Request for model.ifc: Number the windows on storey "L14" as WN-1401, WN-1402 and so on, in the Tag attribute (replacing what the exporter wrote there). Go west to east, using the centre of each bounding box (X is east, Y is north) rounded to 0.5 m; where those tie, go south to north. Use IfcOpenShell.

First a look at what the model holds.

```python
import ifcopenshell
import ifcopenshell.util.element
import ifcopenshell.util.placement

model = ifcopenshell.open("model.ifc")
print(model.schema)
storey = next(s for s in model.by_type("IfcBuildingStorey") if s.Name == "L14")
windows = [e for e in ifcopenshell.util.element.get_decomposition(storey) if e.is_a("IfcWindow")]
for e in sorted(windows, key=lambda e: e.id()):
    origin = ifcopenshell.util.placement.get_local_placement(e.ObjectPlacement)[:3, 3]
    print(e.id(), e.Tag, e.Name, origin.round(2) + 0.0, sep=" | ")
```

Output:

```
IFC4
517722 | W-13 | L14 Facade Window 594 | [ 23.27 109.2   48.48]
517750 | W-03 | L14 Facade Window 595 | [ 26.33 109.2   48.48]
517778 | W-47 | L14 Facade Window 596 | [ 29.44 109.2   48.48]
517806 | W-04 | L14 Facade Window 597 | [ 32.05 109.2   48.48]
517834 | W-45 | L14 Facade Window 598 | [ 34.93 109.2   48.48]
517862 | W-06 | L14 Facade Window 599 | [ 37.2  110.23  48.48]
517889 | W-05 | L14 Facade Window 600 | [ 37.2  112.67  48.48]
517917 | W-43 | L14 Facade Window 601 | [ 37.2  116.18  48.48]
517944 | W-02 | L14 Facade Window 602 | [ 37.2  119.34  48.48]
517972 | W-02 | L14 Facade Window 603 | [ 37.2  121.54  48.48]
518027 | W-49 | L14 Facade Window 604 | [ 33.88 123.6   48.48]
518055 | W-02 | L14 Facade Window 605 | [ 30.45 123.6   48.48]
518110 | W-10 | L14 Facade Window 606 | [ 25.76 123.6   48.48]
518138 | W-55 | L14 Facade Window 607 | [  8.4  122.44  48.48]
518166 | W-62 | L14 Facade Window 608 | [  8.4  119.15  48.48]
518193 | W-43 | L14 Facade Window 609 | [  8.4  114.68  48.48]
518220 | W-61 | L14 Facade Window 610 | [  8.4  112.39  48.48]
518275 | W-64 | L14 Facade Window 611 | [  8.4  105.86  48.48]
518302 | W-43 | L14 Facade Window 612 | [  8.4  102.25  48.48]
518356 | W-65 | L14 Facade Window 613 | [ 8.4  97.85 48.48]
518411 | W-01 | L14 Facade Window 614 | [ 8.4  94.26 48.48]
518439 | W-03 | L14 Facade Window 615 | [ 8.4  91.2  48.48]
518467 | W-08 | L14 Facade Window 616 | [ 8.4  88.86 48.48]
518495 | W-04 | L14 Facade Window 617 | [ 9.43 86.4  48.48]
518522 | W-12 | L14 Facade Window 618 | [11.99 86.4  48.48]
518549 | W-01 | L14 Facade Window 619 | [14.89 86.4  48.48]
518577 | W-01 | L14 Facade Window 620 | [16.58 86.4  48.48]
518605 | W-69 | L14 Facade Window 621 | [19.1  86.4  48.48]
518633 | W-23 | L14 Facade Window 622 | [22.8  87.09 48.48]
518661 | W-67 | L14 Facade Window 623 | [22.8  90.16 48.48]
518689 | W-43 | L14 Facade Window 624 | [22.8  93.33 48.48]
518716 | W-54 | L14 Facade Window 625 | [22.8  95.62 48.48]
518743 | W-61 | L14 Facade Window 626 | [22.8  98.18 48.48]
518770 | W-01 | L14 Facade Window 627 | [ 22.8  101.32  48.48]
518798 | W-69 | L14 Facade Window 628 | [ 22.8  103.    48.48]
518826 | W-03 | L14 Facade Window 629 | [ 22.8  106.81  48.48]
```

```python
import ifcopenshell
import ifcopenshell.geom
import ifcopenshell.util.element
import ifcopenshell.util.shape

model = ifcopenshell.open("model.ifc")
settings = ifcopenshell.geom.settings()
settings.set("use-world-coords", True)


def centre(element):
    shape = ifcopenshell.geom.create_shape(settings, element)
    return ifcopenshell.util.shape.get_bbox_centroid(shape.geometry)


storey = next(s for s in model.by_type("IfcBuildingStorey") if s.Name == "L14")
windows = [e for e in ifcopenshell.util.element.get_decomposition(storey) if e.is_a("IfcWindow")]

# Insertion points can sit at a corner or the storey origin, so sort by the geometry (in metres).
centres = {e: centre(e) for e in windows}
windows.sort(key=lambda e: (round(centres[e][0] / 0.5), centres[e][1]))

for i, e in enumerate(windows, start=1):
    number = f"WN-14{i:02d}"
    e.Tag = number
    print(e.id(), number)

model.write("model_edited.ifc")
```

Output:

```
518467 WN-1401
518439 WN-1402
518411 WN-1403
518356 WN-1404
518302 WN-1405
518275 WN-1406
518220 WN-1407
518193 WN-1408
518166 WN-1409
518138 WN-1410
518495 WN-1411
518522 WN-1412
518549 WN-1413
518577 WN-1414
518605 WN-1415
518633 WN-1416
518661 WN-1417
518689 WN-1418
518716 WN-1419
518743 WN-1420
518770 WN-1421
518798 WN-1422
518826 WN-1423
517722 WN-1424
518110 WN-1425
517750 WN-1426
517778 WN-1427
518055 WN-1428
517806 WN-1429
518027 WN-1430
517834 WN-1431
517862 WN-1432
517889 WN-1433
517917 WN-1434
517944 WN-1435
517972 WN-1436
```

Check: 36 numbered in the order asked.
